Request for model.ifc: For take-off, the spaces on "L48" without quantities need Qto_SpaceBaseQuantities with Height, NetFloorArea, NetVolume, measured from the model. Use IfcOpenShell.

First a look at what the model holds.

```python
import ifcopenshell
import ifcopenshell.util.element
import ifcopenshell.util.unit

model = ifcopenshell.open("model.ifc")
print(model.schema)
for unit_type in ("LENGTHUNIT", "AREAUNIT", "VOLUMEUNIT"):
    print(unit_type, ifcopenshell.util.unit.calculate_unit_scale(model, unit_type))
storey = next(s for s in model.by_type("IfcBuildingStorey") if s.Name == "L48")
spaces = [e for e in ifcopenshell.util.element.get_decomposition(storey) if e.is_a("IfcSpace")]
for e in sorted(spaces, key=lambda e: e.id()):
    print(e.id(), e.is_a(), e.Name, list(ifcopenshell.util.element.get_psets(e, qtos_only=True)), sep=" | ")
```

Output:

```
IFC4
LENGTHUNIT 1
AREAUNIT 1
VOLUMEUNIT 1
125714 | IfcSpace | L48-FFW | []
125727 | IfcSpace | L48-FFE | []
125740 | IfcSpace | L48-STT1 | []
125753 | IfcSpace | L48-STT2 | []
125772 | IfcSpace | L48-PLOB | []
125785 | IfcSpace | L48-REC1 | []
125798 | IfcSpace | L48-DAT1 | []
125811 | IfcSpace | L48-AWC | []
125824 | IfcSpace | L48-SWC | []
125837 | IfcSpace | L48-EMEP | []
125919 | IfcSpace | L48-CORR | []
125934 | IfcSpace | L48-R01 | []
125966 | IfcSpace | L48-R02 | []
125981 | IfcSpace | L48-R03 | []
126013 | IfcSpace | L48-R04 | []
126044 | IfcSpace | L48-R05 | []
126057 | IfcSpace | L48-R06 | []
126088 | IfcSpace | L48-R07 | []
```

```python
import ifcopenshell
import ifcopenshell.api.pset
import ifcopenshell.geom
import ifcopenshell.util.element
import ifcopenshell.util.shape
import ifcopenshell.util.unit

model = ifcopenshell.open("model.ifc")
unit_scale = ifcopenshell.util.unit.calculate_unit_scale(model)
area_scale = ifcopenshell.util.unit.calculate_unit_scale(model, "AREAUNIT")
volume_scale = ifcopenshell.util.unit.calculate_unit_scale(model, "VOLUMEUNIT")
settings = ifcopenshell.geom.settings()

storey = next(s for s in model.by_type("IfcBuildingStorey") if s.Name == "L48")
spaces = [e for e in ifcopenshell.util.element.get_decomposition(storey) if e.is_a("IfcSpace")]

for e in sorted(spaces, key=lambda e: e.id()):
    if ifcopenshell.util.element.get_psets(e, qtos_only=True, should_inherit=False):
        continue
    # Geometry comes back in metres, in the element's own axes.
    shape = ifcopenshell.geom.create_shape(settings, e)
    values = {
        "Height": ifcopenshell.util.shape.get_z(shape.geometry) / unit_scale,
        "NetFloorArea": ifcopenshell.util.shape.get_footprint_area(shape.geometry) / area_scale,
        "NetVolume": ifcopenshell.util.shape.get_volume(shape.geometry) / volume_scale,
    }
    qto = ifcopenshell.api.pset.add_qto(model, product=e, name="Qto_SpaceBaseQuantities")
    ifcopenshell.api.pset.edit_qto(model, qto=qto, properties=values)
    print(e.id(), {k: round(v, 3) for k, v in values.items()})

model.write("model-out.ifc")
```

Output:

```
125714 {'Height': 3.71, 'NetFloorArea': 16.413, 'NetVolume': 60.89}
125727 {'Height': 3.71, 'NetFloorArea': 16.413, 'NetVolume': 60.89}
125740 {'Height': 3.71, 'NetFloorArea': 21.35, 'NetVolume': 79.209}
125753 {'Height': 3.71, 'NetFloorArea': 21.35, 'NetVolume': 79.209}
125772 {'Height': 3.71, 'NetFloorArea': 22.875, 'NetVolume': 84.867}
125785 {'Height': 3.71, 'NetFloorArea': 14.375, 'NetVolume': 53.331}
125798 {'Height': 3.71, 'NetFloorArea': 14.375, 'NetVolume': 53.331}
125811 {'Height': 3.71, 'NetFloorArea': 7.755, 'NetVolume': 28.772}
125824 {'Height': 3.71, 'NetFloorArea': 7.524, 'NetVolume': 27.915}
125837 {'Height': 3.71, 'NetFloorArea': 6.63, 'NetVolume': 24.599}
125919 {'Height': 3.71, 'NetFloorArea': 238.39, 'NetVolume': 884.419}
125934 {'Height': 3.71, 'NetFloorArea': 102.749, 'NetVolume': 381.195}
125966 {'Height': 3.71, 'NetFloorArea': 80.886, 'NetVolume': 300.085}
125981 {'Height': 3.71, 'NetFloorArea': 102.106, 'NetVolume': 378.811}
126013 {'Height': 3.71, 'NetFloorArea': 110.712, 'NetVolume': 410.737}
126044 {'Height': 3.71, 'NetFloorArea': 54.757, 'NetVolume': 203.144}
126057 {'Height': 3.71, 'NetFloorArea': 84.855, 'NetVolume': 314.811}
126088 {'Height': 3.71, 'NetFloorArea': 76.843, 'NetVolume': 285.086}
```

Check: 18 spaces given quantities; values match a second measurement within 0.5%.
